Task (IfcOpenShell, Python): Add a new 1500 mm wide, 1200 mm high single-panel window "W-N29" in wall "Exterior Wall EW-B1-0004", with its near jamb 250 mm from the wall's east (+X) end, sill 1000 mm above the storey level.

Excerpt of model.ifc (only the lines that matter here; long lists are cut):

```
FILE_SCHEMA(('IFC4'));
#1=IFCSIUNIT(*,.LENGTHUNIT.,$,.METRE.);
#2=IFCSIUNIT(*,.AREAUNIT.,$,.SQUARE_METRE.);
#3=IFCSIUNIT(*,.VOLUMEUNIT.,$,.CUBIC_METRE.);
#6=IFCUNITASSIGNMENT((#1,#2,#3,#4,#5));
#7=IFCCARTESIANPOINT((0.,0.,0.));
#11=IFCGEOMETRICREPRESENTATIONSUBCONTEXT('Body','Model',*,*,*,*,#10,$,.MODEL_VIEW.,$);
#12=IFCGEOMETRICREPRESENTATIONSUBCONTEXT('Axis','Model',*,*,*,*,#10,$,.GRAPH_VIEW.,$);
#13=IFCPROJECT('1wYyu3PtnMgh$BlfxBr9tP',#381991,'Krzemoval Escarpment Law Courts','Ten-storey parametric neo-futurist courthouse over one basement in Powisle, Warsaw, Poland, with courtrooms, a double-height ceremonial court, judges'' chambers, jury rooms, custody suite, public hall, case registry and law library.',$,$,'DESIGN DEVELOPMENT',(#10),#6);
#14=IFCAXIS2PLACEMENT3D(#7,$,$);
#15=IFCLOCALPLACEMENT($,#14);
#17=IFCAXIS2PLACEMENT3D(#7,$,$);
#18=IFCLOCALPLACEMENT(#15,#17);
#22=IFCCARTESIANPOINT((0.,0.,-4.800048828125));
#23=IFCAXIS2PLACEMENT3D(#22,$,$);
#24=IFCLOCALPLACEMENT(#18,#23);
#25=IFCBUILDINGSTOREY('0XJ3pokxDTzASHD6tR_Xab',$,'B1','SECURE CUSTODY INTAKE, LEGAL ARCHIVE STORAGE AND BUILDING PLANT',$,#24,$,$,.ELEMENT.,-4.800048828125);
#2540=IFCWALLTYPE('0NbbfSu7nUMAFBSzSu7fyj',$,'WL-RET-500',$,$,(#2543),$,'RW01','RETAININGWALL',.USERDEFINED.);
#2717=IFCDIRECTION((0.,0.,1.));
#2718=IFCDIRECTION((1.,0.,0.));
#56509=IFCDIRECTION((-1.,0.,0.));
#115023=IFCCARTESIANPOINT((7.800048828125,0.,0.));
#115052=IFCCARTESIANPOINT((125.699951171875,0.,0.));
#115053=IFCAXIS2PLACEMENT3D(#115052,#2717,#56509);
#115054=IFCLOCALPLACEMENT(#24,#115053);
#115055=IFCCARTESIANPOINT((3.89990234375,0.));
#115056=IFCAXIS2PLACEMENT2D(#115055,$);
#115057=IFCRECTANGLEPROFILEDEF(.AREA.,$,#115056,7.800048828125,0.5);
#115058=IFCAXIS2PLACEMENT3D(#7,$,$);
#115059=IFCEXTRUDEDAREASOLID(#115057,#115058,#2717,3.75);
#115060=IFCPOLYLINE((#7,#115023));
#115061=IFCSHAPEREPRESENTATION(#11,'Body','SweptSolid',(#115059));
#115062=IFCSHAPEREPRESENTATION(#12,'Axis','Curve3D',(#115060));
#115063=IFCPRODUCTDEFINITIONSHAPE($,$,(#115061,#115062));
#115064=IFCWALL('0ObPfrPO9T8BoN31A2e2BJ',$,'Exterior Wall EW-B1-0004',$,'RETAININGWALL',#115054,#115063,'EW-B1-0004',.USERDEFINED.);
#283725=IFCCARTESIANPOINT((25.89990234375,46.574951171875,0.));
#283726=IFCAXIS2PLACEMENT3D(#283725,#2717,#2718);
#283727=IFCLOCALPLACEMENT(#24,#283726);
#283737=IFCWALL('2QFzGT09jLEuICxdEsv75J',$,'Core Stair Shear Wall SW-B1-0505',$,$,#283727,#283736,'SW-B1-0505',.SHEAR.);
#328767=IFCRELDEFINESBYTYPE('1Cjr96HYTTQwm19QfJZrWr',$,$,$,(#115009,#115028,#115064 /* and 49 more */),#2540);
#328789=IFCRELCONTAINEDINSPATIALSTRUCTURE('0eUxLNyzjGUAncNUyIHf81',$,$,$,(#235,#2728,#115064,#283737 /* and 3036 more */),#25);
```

```python
import numpy as np
import ifcopenshell
import ifcopenshell.api.feature
import ifcopenshell.api.geometry
import ifcopenshell.api.root
import ifcopenshell.api.spatial
import ifcopenshell.geom
import ifcopenshell.util.element
import ifcopenshell.util.placement
import ifcopenshell.util.representation
import ifcopenshell.util.shape
import ifcopenshell.util.unit

model = ifcopenshell.open("model.ifc")
unit_scale = ifcopenshell.util.unit.calculate_unit_scale(model)
settings = ifcopenshell.geom.settings()


def volume(element):
    """Net volume in cubic metres, openings subtracted."""
    shape = ifcopenshell.geom.create_shape(settings, element)
    return ifcopenshell.util.shape.get_volume(shape.geometry)


wall = model.by_guid("0ObPfrPO9T8BoN31A2e2BJ")
storey = ifcopenshell.util.element.get_container(wall, ifc_class="IfcBuildingStorey")
context = ifcopenshell.util.representation.get_context(model, "Model", "Body", "MODEL_VIEW")
before = volume(wall)

width, height, from_end, sill = 1.5, 1.2, 0.25, 1  # metres

# The wall runs along its own X axis, and the end named is its -X end.
wall_shape = ifcopenshell.geom.create_shape(settings, wall)
x, y, z = ifcopenshell.util.shape.get_vertices(wall_shape.geometry).T
start = x.min() + from_end
face, thickness = float(y.min()), float(y.max() - y.min())
wall_matrix = ifcopenshell.util.placement.get_local_placement(wall.ObjectPlacement)
level = ifcopenshell.util.placement.get_local_placement(storey.ObjectPlacement)[2, 3]


def in_wall(x, y):
    """Placement at x, y metres in the wall's axes, at sill height."""
    matrix = wall_matrix.copy()
    matrix[:, 3] = wall_matrix @ np.array([x / unit_scale, y / unit_scale, 0.0, 1.0])
    matrix[2, 3] = level + sill / unit_scale
    return matrix


# Opening: a box that overshoots both wall faces by 50 mm.
opening = ifcopenshell.api.root.create_entity(model, ifc_class="IfcOpeningElement", predefined_type="OPENING")
box = ifcopenshell.api.geometry.add_wall_representation(
    model, context=context, length=width, height=height, thickness=thickness + 0.1
)
ifcopenshell.api.geometry.assign_representation(model, product=opening, representation=box)
ifcopenshell.api.geometry.edit_object_placement(model, product=opening, matrix=in_wall(start, face - 0.05), is_si=False)
ifcopenshell.api.feature.add_feature(model, feature=opening, element=wall)

window = ifcopenshell.api.root.create_entity(model, ifc_class="IfcWindow", name="W-N29", predefined_type="WINDOW")
window.OverallWidth, window.OverallHeight = width / unit_scale, height / unit_scale
window.PartitioningType = "SINGLE_PANEL"
body = ifcopenshell.api.geometry.add_window_representation(
    model,
    context=context,
    overall_width=window.OverallWidth,
    overall_height=window.OverallHeight,
    partition_type="SINGLE_PANEL",
)
ifcopenshell.api.geometry.assign_representation(model, product=window, representation=body)
ifcopenshell.api.spatial.assign_container(model, products=[window], relating_structure=storey)
ifcopenshell.api.feature.add_filling(model, opening=opening, element=window)

# Centre the window in the wall's thickness.
ifcopenshell.api.geometry.edit_object_placement(model, product=window, matrix=in_wall(start, face), is_si=False)
window_shape = ifcopenshell.geom.create_shape(settings, window)
depth = ifcopenshell.util.shape.get_vertices(window_shape.geometry)[:, 1]
offset = face + thickness / 2 - (depth.min() + depth.max()) / 2
ifcopenshell.api.geometry.edit_object_placement(model, product=window, matrix=in_wall(start, offset), is_si=False)

after = volume(wall)

print(f"wall volume {before:.3f} -> {after:.3f} m3")

model.write("model_v2.ifc")
```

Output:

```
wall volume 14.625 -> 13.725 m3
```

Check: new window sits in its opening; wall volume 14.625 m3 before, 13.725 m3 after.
